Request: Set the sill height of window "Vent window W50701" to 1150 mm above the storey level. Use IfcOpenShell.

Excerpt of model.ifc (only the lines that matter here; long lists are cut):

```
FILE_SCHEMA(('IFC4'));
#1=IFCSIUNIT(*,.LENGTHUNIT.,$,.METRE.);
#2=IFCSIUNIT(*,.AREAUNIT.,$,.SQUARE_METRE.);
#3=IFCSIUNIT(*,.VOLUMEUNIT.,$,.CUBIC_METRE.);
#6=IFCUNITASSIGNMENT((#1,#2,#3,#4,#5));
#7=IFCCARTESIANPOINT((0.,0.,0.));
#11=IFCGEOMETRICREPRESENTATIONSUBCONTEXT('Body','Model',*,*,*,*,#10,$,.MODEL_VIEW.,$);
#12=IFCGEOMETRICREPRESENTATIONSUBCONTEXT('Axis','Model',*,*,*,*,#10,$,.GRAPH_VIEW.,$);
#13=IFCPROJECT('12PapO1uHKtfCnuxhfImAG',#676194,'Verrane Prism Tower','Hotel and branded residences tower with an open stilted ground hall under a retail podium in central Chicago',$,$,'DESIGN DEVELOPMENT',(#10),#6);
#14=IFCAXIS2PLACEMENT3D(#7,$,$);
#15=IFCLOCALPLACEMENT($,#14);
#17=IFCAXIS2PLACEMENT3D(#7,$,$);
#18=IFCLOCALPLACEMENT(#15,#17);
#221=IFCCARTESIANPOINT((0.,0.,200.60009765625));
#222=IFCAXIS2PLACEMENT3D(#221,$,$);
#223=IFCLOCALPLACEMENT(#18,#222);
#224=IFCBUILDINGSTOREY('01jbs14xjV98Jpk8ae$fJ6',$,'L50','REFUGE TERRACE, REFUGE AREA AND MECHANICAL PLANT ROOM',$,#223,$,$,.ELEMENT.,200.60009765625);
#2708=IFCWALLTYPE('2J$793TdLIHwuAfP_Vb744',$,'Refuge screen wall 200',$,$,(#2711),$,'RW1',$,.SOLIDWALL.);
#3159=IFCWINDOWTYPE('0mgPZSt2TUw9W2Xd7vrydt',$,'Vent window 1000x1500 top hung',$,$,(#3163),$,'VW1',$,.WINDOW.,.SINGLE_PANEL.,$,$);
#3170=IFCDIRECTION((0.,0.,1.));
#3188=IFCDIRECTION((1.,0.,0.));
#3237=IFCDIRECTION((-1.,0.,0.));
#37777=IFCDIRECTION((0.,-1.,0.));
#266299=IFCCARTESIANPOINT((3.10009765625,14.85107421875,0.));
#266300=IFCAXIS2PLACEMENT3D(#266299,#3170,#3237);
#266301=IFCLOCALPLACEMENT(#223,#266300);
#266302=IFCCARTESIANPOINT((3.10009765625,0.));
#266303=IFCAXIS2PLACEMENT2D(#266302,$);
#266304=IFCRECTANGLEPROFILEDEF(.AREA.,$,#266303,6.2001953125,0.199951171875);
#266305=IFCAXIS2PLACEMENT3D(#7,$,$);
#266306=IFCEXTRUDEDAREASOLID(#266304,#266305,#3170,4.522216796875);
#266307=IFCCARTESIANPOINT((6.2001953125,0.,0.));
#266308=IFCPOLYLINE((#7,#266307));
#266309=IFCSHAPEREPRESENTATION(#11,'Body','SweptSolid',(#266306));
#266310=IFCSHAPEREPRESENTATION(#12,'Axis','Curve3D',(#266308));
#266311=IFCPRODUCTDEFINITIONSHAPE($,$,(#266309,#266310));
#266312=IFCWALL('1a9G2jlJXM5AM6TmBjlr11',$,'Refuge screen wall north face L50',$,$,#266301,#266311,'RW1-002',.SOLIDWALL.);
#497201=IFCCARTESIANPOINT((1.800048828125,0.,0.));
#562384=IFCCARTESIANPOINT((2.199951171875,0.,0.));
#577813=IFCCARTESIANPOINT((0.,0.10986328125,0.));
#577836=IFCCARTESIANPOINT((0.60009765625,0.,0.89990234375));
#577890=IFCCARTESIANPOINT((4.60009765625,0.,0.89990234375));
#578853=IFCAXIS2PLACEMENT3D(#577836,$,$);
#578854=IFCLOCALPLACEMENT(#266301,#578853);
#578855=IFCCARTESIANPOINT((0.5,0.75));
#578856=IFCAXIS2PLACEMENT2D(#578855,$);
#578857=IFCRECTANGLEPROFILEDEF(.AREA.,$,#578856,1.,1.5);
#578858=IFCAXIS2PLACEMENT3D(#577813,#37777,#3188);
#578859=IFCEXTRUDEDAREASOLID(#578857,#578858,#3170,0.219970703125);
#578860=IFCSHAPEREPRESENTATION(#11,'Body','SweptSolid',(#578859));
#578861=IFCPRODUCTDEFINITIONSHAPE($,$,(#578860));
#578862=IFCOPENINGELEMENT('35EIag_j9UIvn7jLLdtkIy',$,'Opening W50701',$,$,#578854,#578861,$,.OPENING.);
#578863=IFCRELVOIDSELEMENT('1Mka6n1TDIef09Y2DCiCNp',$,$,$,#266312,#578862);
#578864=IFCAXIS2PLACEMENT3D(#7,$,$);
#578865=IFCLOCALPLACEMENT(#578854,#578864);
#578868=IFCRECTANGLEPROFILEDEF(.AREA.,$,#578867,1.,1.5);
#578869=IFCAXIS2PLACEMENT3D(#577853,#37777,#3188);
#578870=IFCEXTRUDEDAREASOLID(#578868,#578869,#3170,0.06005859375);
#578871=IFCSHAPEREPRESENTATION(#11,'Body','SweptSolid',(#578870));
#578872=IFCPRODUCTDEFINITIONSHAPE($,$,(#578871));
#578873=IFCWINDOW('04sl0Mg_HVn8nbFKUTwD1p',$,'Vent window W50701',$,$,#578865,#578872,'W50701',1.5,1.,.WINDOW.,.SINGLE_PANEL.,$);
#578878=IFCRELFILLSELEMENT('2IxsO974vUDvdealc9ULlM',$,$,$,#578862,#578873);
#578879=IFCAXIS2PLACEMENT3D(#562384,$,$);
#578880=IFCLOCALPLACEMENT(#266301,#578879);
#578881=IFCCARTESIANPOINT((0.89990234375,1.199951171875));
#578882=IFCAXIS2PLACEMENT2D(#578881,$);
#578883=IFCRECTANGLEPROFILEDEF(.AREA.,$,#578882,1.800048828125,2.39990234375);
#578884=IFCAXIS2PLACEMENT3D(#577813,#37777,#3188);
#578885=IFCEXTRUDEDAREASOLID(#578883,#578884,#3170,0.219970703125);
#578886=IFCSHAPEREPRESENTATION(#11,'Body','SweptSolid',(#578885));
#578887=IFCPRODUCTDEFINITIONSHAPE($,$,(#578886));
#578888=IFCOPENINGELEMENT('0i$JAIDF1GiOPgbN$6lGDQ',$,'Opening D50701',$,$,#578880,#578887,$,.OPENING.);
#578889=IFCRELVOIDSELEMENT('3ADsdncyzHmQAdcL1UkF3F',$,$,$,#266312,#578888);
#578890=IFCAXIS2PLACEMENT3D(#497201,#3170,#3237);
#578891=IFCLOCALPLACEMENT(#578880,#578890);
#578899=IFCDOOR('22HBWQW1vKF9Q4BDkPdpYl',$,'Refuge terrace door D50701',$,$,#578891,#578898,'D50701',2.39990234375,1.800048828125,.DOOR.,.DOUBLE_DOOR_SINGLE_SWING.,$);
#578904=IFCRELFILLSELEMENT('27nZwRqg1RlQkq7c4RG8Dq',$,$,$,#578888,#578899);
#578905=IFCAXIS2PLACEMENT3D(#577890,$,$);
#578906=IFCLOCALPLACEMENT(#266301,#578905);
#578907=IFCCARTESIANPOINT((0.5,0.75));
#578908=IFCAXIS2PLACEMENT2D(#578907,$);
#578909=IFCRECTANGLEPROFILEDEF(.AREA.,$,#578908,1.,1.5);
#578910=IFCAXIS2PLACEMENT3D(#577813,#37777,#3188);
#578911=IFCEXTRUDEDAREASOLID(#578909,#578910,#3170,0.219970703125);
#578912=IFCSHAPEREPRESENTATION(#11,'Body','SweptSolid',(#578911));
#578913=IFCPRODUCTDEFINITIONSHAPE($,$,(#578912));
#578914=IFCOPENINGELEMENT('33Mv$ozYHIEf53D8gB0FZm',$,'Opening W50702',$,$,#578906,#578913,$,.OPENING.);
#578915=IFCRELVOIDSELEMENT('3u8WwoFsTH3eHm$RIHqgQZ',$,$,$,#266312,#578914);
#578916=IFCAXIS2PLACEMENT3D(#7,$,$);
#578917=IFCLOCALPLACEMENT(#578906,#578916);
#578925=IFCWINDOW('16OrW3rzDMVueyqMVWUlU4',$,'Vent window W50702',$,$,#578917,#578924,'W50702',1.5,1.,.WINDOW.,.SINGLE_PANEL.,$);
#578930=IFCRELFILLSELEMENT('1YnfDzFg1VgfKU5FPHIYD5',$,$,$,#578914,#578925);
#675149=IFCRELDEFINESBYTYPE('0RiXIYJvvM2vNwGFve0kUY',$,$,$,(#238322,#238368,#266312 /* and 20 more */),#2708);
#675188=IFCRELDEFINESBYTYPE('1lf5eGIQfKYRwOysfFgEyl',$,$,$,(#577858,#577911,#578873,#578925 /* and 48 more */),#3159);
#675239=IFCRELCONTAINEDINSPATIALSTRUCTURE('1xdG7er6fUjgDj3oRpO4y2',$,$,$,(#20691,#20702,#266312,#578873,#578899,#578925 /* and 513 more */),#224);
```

```python
import numpy as np
import ifcopenshell
import ifcopenshell.api.geometry
import ifcopenshell.geom
import ifcopenshell.util.element
import ifcopenshell.util.placement
import ifcopenshell.util.shape
import ifcopenshell.util.unit

model = ifcopenshell.open("model.ifc")
unit_scale = ifcopenshell.util.unit.calculate_unit_scale(model)

window = model.by_guid("04sl0Mg_HVn8nbFKUTwD1p")
opening = window.FillsVoids[0].RelatingOpeningElement
storey = ifcopenshell.util.element.get_container(window, ifc_class="IfcBuildingStorey")
level = ifcopenshell.util.placement.get_local_placement(storey.ObjectPlacement)[2, 3]

# The opening's origin need not be at the sill, so measure its lowest point.
shape = ifcopenshell.geom.create_shape(ifcopenshell.geom.settings(), opening)
bottom = ifcopenshell.util.shape.get_shape_bottom_elevation(shape, shape.geometry) / unit_scale
dz = level + 1.15 / unit_scale - bottom

shift = np.array([0.0, 0.0, dz])
# The window is placed relative to its opening, so it follows when the opening moves.
matrix = ifcopenshell.util.placement.get_local_placement(opening.ObjectPlacement)
matrix[:3, 3] += shift
ifcopenshell.api.geometry.edit_object_placement(
    model, product=opening, matrix=matrix, is_si=False, should_transform_children=True
)

print(f"moved by {dz * unit_scale:+.3f} m")

model.write("model_v2.ifc")
```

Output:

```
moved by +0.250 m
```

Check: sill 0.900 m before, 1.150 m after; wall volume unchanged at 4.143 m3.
